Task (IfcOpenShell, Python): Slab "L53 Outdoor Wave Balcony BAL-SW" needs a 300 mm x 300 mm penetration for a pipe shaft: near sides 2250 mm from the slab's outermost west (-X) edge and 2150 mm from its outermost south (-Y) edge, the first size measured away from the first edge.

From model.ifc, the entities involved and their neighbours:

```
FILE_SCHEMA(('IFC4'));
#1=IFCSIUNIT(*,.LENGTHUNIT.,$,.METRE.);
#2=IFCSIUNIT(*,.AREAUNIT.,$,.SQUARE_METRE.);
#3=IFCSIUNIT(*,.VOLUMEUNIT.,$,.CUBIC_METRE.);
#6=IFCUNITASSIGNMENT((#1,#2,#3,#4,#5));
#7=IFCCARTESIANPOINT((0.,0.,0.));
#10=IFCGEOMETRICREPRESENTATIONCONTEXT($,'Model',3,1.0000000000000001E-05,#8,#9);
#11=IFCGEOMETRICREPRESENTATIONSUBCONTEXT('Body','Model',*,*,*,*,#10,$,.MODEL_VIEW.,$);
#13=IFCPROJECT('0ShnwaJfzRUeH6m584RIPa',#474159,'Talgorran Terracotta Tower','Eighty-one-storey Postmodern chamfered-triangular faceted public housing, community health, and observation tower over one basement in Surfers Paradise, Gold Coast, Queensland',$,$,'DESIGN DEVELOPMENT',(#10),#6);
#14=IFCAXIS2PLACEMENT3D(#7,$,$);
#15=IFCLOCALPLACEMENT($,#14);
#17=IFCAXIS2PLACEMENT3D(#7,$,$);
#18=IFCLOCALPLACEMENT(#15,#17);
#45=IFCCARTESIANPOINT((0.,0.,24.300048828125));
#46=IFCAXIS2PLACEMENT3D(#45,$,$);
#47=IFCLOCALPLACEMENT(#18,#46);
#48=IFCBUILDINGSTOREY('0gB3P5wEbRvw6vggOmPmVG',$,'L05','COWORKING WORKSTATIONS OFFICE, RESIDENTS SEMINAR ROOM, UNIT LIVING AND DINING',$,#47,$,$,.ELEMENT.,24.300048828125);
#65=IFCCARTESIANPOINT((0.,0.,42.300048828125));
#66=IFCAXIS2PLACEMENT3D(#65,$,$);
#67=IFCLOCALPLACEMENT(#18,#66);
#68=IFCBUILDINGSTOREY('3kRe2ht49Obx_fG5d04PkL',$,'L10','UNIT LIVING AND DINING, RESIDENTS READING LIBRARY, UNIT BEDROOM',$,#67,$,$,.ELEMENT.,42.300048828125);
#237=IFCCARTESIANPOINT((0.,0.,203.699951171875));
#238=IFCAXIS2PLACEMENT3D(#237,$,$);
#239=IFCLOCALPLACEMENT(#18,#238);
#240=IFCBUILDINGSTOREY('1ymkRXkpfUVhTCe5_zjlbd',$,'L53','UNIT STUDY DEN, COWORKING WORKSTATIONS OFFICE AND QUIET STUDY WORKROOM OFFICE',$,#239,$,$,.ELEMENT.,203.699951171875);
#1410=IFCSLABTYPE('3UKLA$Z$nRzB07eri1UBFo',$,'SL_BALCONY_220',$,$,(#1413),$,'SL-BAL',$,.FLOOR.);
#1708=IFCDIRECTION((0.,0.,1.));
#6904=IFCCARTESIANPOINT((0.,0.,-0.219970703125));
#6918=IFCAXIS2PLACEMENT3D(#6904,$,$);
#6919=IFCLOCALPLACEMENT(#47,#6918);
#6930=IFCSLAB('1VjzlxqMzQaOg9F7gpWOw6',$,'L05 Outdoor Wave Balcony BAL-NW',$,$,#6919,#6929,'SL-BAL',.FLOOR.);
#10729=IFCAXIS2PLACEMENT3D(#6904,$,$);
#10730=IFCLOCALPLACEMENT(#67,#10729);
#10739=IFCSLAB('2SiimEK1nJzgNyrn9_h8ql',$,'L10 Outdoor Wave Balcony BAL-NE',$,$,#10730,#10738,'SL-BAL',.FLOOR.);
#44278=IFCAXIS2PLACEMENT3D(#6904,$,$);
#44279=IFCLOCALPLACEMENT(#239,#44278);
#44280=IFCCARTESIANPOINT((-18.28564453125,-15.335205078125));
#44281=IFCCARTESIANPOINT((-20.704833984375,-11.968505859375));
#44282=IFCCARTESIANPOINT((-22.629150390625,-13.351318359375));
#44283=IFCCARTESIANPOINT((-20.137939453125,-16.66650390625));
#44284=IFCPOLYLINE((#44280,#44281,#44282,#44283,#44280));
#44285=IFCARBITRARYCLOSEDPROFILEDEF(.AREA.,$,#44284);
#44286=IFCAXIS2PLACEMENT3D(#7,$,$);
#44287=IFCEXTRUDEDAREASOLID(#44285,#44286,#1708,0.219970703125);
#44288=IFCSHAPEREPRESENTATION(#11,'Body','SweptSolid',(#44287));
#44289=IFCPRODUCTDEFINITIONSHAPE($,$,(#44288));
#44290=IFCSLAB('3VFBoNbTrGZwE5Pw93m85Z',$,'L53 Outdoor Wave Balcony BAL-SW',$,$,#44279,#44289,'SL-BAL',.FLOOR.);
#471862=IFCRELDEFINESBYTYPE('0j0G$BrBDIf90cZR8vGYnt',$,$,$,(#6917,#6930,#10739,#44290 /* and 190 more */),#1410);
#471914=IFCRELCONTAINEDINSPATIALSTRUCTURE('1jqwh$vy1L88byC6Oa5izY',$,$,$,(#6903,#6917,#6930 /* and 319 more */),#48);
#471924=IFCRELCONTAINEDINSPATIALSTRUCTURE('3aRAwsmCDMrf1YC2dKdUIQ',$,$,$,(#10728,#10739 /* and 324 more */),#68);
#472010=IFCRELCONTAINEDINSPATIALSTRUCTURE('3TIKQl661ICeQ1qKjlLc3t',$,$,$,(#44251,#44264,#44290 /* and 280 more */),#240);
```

```python
import numpy as np
import ifcopenshell
import ifcopenshell.api.feature
import ifcopenshell.api.geometry
import ifcopenshell.api.root
import ifcopenshell.geom
import ifcopenshell.util.placement
import ifcopenshell.util.representation
import ifcopenshell.util.shape
import ifcopenshell.util.unit

model = ifcopenshell.open("model.ifc")
unit_scale = ifcopenshell.util.unit.calculate_unit_scale(model)
settings = ifcopenshell.geom.settings()


def volume(element):
    """Net volume in cubic metres, openings subtracted."""
    shape = ifcopenshell.geom.create_shape(settings, element)
    return ifcopenshell.util.shape.get_volume(shape.geometry)


slab = model.by_guid("3VFBoNbTrGZwE5Pw93m85Z")
before = volume(slab)

# Extent in the slab's own axes, in metres. The edges named are its -X and -Y sides.
slab_shape = ifcopenshell.geom.create_shape(settings, slab)
vertices = ifcopenshell.util.shape.get_vertices(slab_shape.geometry)
x_min, y_min, bottom = vertices.min(axis=0)
top = vertices[:, 2].max()

opening = ifcopenshell.api.root.create_entity(model, ifc_class="IfcOpeningElement", name="Pipe shaft opening", predefined_type="OPENING")
context = ifcopenshell.util.representation.get_context(model, "Model", "Body", "MODEL_VIEW")
width, depth = 0.3, 0.3
outline = [(0.0, 0.0), (width, 0.0), (width, depth), (0.0, depth), (0.0, 0.0)]
# Overshoot both faces by 50 mm so the cut is clean.
shape = ifcopenshell.api.geometry.add_slab_representation(
    model, context=context, depth=top - bottom + 0.1, polyline=outline
)
ifcopenshell.api.geometry.assign_representation(model, product=opening, representation=shape)

matrix = ifcopenshell.util.placement.get_local_placement(slab.ObjectPlacement)
matrix[:, 3] = matrix @ np.append(np.array([x_min + 2.25, y_min + 2.15, bottom - 0.05]) / unit_scale, 1.0)
ifcopenshell.api.geometry.edit_object_placement(model, product=opening, matrix=matrix, is_si=False)
ifcopenshell.api.feature.add_feature(model, feature=opening, element=slab)

after = volume(slab)

print(f"slab volume {before:.3f} -> {after:.3f} m3")

model.write("model_edited.ifc")
```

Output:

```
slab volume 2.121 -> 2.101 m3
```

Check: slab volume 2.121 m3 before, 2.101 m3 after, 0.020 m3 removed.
